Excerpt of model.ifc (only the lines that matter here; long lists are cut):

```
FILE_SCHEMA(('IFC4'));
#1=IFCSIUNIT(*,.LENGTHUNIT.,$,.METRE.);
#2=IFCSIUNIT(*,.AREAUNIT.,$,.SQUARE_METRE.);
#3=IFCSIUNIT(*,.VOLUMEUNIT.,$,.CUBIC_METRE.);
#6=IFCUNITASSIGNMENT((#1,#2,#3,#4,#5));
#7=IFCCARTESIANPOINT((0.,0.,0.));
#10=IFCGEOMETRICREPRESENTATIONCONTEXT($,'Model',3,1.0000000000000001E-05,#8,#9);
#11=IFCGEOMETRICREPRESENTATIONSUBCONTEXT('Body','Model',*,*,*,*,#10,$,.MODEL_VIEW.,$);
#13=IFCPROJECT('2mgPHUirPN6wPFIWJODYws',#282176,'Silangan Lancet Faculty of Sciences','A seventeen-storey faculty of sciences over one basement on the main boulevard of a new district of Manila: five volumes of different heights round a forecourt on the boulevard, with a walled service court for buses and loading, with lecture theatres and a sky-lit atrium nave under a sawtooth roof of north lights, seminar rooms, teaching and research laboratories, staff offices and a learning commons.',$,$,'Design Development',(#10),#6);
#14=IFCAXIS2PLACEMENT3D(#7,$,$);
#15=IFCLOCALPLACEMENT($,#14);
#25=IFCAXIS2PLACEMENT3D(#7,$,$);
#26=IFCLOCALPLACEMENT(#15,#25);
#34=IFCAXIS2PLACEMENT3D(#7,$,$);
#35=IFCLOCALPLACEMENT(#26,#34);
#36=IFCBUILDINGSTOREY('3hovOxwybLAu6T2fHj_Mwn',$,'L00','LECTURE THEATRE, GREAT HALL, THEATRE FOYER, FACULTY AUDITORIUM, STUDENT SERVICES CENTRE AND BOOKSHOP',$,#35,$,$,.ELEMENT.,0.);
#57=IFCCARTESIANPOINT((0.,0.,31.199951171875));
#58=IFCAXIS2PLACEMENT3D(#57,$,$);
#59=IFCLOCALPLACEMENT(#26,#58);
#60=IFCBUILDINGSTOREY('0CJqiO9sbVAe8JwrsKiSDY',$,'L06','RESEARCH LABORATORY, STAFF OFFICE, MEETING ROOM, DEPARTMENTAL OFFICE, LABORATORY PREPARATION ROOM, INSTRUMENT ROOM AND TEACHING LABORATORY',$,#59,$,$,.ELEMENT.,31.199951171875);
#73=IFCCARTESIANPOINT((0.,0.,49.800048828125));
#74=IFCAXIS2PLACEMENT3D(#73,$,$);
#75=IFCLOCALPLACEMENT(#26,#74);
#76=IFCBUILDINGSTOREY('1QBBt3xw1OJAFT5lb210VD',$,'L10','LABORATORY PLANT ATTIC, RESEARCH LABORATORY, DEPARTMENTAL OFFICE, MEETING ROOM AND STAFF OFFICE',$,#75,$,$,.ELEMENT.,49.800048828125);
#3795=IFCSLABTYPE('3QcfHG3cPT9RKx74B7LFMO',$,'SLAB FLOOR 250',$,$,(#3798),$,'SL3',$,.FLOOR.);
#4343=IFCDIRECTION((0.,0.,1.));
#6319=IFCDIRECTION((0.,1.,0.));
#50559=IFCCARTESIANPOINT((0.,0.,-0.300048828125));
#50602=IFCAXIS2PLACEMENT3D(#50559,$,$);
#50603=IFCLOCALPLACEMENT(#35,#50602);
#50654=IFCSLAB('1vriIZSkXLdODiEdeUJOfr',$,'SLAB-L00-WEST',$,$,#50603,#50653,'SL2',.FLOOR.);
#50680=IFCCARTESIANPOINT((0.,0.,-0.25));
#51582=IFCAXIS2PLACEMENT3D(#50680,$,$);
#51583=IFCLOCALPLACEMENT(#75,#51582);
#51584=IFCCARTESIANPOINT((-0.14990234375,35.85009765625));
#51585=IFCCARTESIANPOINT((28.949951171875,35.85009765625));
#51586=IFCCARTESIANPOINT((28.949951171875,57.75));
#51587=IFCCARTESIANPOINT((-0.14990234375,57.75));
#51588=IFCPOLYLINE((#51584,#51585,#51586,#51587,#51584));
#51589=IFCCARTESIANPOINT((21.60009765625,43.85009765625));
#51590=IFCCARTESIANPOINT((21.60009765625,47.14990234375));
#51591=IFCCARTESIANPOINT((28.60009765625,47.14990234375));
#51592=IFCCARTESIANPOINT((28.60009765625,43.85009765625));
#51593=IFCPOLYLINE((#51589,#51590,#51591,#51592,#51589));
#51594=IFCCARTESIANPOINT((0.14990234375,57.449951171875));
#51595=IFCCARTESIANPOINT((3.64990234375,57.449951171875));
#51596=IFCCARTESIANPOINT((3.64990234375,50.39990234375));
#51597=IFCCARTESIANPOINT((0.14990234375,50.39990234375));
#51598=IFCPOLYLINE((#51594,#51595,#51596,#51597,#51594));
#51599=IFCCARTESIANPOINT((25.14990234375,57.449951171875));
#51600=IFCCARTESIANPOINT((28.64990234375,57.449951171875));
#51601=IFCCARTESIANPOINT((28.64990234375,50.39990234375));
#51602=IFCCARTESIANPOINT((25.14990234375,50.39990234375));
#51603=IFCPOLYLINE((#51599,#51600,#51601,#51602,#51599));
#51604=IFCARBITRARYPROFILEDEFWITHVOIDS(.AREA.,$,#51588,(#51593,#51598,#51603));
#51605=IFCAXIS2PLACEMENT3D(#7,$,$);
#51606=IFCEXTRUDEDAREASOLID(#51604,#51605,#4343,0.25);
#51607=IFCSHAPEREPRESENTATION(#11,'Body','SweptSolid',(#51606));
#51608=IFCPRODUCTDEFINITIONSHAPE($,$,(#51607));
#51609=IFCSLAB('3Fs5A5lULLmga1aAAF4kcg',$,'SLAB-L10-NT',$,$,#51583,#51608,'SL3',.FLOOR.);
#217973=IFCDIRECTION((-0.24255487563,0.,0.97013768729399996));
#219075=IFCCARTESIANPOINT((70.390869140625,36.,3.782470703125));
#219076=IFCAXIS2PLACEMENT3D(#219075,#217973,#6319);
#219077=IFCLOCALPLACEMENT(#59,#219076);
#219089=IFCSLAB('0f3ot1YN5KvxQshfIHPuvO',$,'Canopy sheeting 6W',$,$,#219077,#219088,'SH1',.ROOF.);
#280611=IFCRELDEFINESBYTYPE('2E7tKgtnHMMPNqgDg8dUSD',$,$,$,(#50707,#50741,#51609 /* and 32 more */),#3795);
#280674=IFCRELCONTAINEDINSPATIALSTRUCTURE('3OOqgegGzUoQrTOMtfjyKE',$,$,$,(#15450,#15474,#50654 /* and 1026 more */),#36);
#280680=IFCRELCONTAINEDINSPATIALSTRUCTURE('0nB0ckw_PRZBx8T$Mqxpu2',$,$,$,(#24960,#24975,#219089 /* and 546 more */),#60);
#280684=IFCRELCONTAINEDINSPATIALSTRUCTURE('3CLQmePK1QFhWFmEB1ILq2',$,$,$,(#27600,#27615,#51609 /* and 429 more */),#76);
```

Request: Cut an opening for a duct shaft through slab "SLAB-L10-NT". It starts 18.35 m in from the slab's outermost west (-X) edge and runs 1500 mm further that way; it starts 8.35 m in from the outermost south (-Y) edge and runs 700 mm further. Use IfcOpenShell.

```python
import numpy as np
import ifcopenshell
import ifcopenshell.api.feature
import ifcopenshell.api.geometry
import ifcopenshell.api.root
import ifcopenshell.geom
import ifcopenshell.util.placement
import ifcopenshell.util.representation
import ifcopenshell.util.shape
import ifcopenshell.util.unit

model = ifcopenshell.open("model.ifc")
unit_scale = ifcopenshell.util.unit.calculate_unit_scale(model)
settings = ifcopenshell.geom.settings()


def volume(element):
    """Net volume in cubic metres, openings subtracted."""
    shape = ifcopenshell.geom.create_shape(settings, element)
    return ifcopenshell.util.shape.get_volume(shape.geometry)


slab = model.by_guid("3Fs5A5lULLmga1aAAF4kcg")
before = volume(slab)

# Extent in the slab's own axes, in metres. The edges named are its -X and -Y sides.
slab_shape = ifcopenshell.geom.create_shape(settings, slab)
vertices = ifcopenshell.util.shape.get_vertices(slab_shape.geometry)
x_min, y_min, bottom = vertices.min(axis=0)
top = vertices[:, 2].max()

opening = ifcopenshell.api.root.create_entity(model, ifc_class="IfcOpeningElement", name="Duct shaft opening", predefined_type="OPENING")
context = ifcopenshell.util.representation.get_context(model, "Model", "Body", "MODEL_VIEW")
width, depth = 1.5, 0.7
outline = [(0.0, 0.0), (width, 0.0), (width, depth), (0.0, depth), (0.0, 0.0)]
# Overshoot both faces by 50 mm so the cut is clean.
shape = ifcopenshell.api.geometry.add_slab_representation(
    model, context=context, depth=top - bottom + 0.1, polyline=outline
)
ifcopenshell.api.geometry.assign_representation(model, product=opening, representation=shape)

matrix = ifcopenshell.util.placement.get_local_placement(slab.ObjectPlacement)
matrix[:, 3] = matrix @ np.append(np.array([x_min + 18.35, y_min + 8.35, bottom - 0.05]) / unit_scale, 1.0)
ifcopenshell.api.geometry.edit_object_placement(model, product=opening, matrix=matrix, is_si=False)
ifcopenshell.api.feature.add_feature(model, feature=opening, element=slab)

after = volume(slab)

print(f"slab volume {before:.3f} -> {after:.3f} m3")

model.write("model_updated.ifc")
```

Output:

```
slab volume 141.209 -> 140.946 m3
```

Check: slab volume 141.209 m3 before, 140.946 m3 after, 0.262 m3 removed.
